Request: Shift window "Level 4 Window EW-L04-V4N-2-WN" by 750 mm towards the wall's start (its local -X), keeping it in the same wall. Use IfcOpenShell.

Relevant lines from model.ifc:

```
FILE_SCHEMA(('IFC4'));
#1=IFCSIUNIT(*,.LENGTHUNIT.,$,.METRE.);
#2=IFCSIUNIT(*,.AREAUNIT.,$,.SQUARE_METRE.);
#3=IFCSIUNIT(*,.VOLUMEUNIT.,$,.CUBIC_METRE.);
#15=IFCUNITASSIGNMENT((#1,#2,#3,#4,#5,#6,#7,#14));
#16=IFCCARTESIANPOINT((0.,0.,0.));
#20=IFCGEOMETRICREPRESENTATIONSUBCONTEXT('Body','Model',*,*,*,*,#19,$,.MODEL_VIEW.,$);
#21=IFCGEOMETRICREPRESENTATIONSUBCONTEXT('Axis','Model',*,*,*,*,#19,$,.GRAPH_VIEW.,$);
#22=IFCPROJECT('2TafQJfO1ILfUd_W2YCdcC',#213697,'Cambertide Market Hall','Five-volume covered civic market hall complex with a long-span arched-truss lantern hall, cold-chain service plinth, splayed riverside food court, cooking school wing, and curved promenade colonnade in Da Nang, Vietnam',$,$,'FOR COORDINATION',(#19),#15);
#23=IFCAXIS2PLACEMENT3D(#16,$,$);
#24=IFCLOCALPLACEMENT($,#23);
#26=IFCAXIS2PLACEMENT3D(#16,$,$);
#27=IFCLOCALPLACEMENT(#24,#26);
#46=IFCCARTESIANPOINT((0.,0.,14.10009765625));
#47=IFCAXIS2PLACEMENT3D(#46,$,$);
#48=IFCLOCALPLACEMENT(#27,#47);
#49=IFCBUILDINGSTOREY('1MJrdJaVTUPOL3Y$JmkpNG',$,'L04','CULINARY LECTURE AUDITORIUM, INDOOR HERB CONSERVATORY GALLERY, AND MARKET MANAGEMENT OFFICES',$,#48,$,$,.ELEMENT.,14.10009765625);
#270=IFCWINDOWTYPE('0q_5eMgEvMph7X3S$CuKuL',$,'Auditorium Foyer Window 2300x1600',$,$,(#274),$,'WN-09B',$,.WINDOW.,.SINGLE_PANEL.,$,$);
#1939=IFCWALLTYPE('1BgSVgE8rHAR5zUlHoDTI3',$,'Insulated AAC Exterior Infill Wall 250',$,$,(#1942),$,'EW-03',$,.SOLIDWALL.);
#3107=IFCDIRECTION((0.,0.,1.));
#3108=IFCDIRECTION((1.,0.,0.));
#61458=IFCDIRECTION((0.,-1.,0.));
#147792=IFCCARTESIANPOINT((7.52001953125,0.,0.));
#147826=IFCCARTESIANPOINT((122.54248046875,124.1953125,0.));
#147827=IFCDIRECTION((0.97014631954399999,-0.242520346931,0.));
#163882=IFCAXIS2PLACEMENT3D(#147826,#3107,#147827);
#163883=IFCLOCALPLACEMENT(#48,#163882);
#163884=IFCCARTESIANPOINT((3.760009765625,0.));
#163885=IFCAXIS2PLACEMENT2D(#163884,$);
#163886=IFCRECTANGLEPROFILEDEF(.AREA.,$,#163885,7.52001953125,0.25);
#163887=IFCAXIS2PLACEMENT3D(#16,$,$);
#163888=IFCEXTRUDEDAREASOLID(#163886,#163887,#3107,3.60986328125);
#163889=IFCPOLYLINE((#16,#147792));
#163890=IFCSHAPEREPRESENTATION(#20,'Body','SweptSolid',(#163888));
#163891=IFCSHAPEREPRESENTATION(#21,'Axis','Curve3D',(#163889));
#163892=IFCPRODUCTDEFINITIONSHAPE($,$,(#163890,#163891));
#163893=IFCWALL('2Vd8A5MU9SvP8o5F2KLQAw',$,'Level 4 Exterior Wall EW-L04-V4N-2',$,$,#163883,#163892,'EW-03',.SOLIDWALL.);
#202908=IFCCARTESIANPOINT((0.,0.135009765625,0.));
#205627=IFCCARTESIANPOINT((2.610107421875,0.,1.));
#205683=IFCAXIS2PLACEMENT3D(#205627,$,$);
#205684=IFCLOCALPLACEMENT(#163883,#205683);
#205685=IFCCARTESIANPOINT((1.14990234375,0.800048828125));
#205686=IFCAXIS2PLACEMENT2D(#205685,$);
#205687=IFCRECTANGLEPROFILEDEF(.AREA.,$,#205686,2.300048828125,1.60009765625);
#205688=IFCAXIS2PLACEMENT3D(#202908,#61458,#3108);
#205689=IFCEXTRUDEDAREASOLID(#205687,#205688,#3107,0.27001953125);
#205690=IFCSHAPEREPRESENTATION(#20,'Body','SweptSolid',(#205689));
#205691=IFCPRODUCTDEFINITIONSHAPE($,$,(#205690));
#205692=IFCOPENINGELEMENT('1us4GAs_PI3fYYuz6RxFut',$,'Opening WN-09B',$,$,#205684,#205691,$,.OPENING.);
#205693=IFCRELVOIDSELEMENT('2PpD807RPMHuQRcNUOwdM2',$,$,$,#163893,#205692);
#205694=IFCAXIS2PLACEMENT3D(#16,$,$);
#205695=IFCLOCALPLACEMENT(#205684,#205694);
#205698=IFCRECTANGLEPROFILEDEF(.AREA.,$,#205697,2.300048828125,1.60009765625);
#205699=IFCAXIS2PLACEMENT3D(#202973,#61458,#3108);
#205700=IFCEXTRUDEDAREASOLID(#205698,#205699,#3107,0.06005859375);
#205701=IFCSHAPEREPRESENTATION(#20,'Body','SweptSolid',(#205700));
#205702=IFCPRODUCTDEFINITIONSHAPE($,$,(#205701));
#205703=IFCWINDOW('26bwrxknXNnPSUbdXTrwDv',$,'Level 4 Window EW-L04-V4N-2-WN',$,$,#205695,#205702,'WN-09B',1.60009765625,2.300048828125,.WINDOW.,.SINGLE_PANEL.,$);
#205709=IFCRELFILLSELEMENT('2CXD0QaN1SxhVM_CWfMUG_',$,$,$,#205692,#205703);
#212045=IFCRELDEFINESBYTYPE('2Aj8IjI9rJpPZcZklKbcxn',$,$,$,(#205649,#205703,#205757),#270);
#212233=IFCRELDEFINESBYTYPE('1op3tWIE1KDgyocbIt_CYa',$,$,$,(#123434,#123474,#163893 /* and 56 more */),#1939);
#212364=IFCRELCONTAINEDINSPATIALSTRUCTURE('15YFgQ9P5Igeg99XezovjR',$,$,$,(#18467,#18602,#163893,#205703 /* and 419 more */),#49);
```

```python
import ifcopenshell
import ifcopenshell.api.geometry
import ifcopenshell.util.placement

model = ifcopenshell.open("model.ifc")

window = model.by_guid("26bwrxknXNnPSUbdXTrwDv")
opening = window.FillsVoids[0].RelatingOpeningElement
wall = opening.VoidsElements[0].RelatingBuildingElement

wall_matrix = ifcopenshell.util.placement.get_local_placement(wall.ObjectPlacement)
shift = wall_matrix[:3, 0] * -0.75
before = ifcopenshell.util.placement.get_local_placement(window.ObjectPlacement)[:3, 3].copy()

# The window is placed relative to its opening, so it follows when the opening moves.
matrix = ifcopenshell.util.placement.get_local_placement(opening.ObjectPlacement)
matrix[:3, 3] += shift
ifcopenshell.api.geometry.edit_object_placement(
    model, product=opening, matrix=matrix, is_si=False, should_transform_children=True
)

after = ifcopenshell.util.placement.get_local_placement(window.ObjectPlacement)[:3, 3]
print("window moved by", (after - before).round(3) + 0.0)

model.write("model_v2.ifc")
```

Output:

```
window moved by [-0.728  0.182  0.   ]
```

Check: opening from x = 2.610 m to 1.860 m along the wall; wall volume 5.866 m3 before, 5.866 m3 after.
